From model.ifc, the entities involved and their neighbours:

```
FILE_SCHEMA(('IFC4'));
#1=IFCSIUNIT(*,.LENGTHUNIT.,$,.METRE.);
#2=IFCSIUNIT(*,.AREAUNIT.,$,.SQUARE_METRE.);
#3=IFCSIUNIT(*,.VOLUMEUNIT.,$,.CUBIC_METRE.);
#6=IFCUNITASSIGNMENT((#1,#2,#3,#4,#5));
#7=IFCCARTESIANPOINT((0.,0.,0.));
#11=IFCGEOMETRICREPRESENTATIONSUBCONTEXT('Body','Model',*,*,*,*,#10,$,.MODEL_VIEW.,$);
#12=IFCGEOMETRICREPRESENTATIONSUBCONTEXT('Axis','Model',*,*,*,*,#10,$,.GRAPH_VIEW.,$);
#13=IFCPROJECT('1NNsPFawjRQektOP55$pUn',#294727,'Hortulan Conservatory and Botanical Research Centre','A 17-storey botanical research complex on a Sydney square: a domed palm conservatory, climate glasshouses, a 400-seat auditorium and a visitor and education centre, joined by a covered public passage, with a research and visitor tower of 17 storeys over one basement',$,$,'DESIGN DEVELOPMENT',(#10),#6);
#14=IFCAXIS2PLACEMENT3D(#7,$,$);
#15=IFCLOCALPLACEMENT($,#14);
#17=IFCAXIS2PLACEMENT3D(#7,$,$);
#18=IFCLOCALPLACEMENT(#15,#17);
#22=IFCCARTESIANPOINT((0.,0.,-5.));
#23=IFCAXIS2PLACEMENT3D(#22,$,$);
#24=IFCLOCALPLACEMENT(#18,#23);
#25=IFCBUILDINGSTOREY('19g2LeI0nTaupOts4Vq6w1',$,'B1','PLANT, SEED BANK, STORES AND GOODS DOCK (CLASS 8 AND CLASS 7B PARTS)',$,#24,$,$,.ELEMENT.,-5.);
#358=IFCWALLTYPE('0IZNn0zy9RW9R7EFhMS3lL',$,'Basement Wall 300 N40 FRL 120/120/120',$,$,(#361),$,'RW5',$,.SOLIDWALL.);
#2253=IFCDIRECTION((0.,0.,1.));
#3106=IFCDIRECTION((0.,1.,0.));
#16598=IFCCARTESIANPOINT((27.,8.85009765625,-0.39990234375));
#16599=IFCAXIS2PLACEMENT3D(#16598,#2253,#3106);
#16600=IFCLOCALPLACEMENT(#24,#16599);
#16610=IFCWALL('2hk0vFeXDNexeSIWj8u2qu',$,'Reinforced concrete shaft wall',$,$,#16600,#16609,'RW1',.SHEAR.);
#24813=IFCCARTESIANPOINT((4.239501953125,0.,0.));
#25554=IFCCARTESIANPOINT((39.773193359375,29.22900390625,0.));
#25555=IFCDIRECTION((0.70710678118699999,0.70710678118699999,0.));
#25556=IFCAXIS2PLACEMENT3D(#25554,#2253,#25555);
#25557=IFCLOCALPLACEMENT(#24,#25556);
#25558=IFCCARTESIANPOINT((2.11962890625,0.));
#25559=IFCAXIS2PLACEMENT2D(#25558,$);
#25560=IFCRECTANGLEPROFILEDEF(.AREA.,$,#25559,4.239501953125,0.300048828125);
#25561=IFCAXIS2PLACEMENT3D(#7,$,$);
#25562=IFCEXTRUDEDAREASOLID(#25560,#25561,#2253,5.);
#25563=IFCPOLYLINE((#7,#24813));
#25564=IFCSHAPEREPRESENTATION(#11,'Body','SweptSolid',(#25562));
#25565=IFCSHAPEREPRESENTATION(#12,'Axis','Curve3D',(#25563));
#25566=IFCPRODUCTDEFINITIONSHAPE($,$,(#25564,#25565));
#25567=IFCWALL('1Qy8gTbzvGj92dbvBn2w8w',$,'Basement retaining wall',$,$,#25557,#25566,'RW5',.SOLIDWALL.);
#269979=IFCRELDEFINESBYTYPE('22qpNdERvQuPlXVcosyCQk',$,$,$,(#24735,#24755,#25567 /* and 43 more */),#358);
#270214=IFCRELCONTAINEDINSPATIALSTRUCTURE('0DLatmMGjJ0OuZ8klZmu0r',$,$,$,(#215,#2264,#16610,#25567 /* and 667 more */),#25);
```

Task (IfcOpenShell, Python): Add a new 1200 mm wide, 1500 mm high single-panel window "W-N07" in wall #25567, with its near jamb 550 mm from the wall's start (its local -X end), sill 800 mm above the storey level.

```python
import numpy as np
import ifcopenshell
import ifcopenshell.api.feature
import ifcopenshell.api.geometry
import ifcopenshell.api.root
import ifcopenshell.api.spatial
import ifcopenshell.geom
import ifcopenshell.util.element
import ifcopenshell.util.placement
import ifcopenshell.util.representation
import ifcopenshell.util.shape
import ifcopenshell.util.unit

model = ifcopenshell.open("model.ifc")
unit_scale = ifcopenshell.util.unit.calculate_unit_scale(model)
settings = ifcopenshell.geom.settings()


def volume(element):
    """Net volume in cubic metres, openings subtracted."""
    shape = ifcopenshell.geom.create_shape(settings, element)
    return ifcopenshell.util.shape.get_volume(shape.geometry)


wall = model.by_guid("1Qy8gTbzvGj92dbvBn2w8w")
storey = ifcopenshell.util.element.get_container(wall, ifc_class="IfcBuildingStorey")
context = ifcopenshell.util.representation.get_context(model, "Model", "Body", "MODEL_VIEW")
before = volume(wall)

width, height, from_end, sill = 1.2, 1.5, 0.55, 0.8  # metres

# The wall runs along its own X axis, and the end named is its -X end.
wall_shape = ifcopenshell.geom.create_shape(settings, wall)
x, y, z = ifcopenshell.util.shape.get_vertices(wall_shape.geometry).T
start = x.min() + from_end
face, thickness = float(y.min()), float(y.max() - y.min())
wall_matrix = ifcopenshell.util.placement.get_local_placement(wall.ObjectPlacement)
level = ifcopenshell.util.placement.get_local_placement(storey.ObjectPlacement)[2, 3]


def in_wall(x, y):
    """Placement at x, y metres in the wall's axes, at sill height."""
    matrix = wall_matrix.copy()
    matrix[:, 3] = wall_matrix @ np.array([x / unit_scale, y / unit_scale, 0.0, 1.0])
    matrix[2, 3] = level + sill / unit_scale
    return matrix


# Opening: a box that overshoots both wall faces by 50 mm.
opening = ifcopenshell.api.root.create_entity(model, ifc_class="IfcOpeningElement", predefined_type="OPENING")
box = ifcopenshell.api.geometry.add_wall_representation(
    model, context=context, length=width, height=height, thickness=thickness + 0.1
)
ifcopenshell.api.geometry.assign_representation(model, product=opening, representation=box)
ifcopenshell.api.geometry.edit_object_placement(model, product=opening, matrix=in_wall(start, face - 0.05), is_si=False)
ifcopenshell.api.feature.add_feature(model, feature=opening, element=wall)

window = ifcopenshell.api.root.create_entity(model, ifc_class="IfcWindow", name="W-N07", predefined_type="WINDOW")
window.OverallWidth, window.OverallHeight = width / unit_scale, height / unit_scale
window.PartitioningType = "SINGLE_PANEL"
body = ifcopenshell.api.geometry.add_window_representation(
    model,
    context=context,
    overall_width=window.OverallWidth,
    overall_height=window.OverallHeight,
    partition_type="SINGLE_PANEL",
)
ifcopenshell.api.geometry.assign_representation(model, product=window, representation=body)
ifcopenshell.api.spatial.assign_container(model, products=[window], relating_structure=storey)
ifcopenshell.api.feature.add_filling(model, opening=opening, element=window)

# Centre the window in the wall's thickness.
ifcopenshell.api.geometry.edit_object_placement(model, product=window, matrix=in_wall(start, face), is_si=False)
window_shape = ifcopenshell.geom.create_shape(settings, window)
depth = ifcopenshell.util.shape.get_vertices(window_shape.geometry)[:, 1]
offset = face + thickness / 2 - (depth.min() + depth.max()) / 2
ifcopenshell.api.geometry.edit_object_placement(model, product=window, matrix=in_wall(start, offset), is_si=False)

after = volume(wall)

print(f"wall volume {before:.3f} -> {after:.3f} m3")

model.write("model_rev.ifc")
```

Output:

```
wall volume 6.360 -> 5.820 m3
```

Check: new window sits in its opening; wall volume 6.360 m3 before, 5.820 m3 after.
